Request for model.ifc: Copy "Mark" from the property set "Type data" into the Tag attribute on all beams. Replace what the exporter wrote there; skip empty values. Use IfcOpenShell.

First a look at what the model holds.

```python
import ifcopenshell
import ifcopenshell.util.element

model = ifcopenshell.open("model.ifc")
print(model.schema)
beams = model.by_type("IfcBeam")
print(len(beams), "beams")
for e in beams[:8]:
    source = ifcopenshell.util.element.get_pset(e, "Type data", "Mark")
    target = e.Tag
    print(e.id(), repr(source), repr(target), sep=" | ")
```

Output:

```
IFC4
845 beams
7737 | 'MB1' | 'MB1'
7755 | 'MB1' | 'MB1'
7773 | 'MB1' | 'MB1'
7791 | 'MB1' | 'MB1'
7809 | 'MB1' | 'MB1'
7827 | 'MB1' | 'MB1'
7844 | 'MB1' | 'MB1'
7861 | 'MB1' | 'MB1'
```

```python
import ifcopenshell
import ifcopenshell.util.element

model = ifcopenshell.open("model.ifc")

count = 0
for e in model.by_type("IfcBeam"):
    value = ifcopenshell.util.element.get_pset(e, "Type data", "Mark")
    current = e.Tag
    if not value or not value.strip() or current == value:
        continue
    e.Tag = value
    count += 1

print(count, "beams updated")

model.write("model_edited.ifc")
```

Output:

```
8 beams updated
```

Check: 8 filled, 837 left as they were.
